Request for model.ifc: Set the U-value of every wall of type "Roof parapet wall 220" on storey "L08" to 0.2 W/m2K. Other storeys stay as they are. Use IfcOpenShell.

First a look at what the model holds.

```python
import ifcopenshell
import ifcopenshell.util.element

model = ifcopenshell.open("model.ifc")
print(model.schema)
storey = next(s for s in model.by_type("IfcBuildingStorey") if s.Name == "L08")
walls = [e for e in ifcopenshell.util.element.get_decomposition(storey) if e.is_a("IfcWall")]
seen = {}
for e in walls:
    element_type = ifcopenshell.util.element.get_type(e)
    key = (element_type.Name if element_type != e and element_type else None, ifcopenshell.util.element.get_pset(e, "Pset_WallCommon", "ThermalTransmittance"))
    seen[key] = seen.get(key, 0) + 1
for (name, value), count in sorted(seen.items(), key=str):
    print(count, "x", name, "|", value)
```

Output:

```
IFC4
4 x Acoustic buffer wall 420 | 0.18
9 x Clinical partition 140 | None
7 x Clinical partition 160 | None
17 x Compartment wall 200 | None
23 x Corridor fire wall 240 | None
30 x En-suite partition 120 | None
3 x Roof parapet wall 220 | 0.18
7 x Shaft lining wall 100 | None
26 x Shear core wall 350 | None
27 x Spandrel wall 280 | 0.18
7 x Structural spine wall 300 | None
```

```python
import ifcopenshell
import ifcopenshell.api.pset
import ifcopenshell.util.element

model = ifcopenshell.open("model.ifc")

storey = next(s for s in model.by_type("IfcBuildingStorey") if s.Name == "L08")
walls = [e for e in ifcopenshell.util.element.get_decomposition(storey) if e.is_a("IfcWall")]

count = 0
for e in walls:
    element_type = ifcopenshell.util.element.get_type(e)
    if element_type in (None, e) or element_type.Name != "Roof parapet wall 220":
        continue
    # add_pset returns the element's existing set when there is one.
    pset = ifcopenshell.api.pset.add_pset(model, product=e, name="Pset_WallCommon")
    ifcopenshell.api.pset.edit_pset(model, pset=pset, properties={"ThermalTransmittance": 0.2})
    count += 1

print(count, "walls updated")

model.write("model-out.ifc")
```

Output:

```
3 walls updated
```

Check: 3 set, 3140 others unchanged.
